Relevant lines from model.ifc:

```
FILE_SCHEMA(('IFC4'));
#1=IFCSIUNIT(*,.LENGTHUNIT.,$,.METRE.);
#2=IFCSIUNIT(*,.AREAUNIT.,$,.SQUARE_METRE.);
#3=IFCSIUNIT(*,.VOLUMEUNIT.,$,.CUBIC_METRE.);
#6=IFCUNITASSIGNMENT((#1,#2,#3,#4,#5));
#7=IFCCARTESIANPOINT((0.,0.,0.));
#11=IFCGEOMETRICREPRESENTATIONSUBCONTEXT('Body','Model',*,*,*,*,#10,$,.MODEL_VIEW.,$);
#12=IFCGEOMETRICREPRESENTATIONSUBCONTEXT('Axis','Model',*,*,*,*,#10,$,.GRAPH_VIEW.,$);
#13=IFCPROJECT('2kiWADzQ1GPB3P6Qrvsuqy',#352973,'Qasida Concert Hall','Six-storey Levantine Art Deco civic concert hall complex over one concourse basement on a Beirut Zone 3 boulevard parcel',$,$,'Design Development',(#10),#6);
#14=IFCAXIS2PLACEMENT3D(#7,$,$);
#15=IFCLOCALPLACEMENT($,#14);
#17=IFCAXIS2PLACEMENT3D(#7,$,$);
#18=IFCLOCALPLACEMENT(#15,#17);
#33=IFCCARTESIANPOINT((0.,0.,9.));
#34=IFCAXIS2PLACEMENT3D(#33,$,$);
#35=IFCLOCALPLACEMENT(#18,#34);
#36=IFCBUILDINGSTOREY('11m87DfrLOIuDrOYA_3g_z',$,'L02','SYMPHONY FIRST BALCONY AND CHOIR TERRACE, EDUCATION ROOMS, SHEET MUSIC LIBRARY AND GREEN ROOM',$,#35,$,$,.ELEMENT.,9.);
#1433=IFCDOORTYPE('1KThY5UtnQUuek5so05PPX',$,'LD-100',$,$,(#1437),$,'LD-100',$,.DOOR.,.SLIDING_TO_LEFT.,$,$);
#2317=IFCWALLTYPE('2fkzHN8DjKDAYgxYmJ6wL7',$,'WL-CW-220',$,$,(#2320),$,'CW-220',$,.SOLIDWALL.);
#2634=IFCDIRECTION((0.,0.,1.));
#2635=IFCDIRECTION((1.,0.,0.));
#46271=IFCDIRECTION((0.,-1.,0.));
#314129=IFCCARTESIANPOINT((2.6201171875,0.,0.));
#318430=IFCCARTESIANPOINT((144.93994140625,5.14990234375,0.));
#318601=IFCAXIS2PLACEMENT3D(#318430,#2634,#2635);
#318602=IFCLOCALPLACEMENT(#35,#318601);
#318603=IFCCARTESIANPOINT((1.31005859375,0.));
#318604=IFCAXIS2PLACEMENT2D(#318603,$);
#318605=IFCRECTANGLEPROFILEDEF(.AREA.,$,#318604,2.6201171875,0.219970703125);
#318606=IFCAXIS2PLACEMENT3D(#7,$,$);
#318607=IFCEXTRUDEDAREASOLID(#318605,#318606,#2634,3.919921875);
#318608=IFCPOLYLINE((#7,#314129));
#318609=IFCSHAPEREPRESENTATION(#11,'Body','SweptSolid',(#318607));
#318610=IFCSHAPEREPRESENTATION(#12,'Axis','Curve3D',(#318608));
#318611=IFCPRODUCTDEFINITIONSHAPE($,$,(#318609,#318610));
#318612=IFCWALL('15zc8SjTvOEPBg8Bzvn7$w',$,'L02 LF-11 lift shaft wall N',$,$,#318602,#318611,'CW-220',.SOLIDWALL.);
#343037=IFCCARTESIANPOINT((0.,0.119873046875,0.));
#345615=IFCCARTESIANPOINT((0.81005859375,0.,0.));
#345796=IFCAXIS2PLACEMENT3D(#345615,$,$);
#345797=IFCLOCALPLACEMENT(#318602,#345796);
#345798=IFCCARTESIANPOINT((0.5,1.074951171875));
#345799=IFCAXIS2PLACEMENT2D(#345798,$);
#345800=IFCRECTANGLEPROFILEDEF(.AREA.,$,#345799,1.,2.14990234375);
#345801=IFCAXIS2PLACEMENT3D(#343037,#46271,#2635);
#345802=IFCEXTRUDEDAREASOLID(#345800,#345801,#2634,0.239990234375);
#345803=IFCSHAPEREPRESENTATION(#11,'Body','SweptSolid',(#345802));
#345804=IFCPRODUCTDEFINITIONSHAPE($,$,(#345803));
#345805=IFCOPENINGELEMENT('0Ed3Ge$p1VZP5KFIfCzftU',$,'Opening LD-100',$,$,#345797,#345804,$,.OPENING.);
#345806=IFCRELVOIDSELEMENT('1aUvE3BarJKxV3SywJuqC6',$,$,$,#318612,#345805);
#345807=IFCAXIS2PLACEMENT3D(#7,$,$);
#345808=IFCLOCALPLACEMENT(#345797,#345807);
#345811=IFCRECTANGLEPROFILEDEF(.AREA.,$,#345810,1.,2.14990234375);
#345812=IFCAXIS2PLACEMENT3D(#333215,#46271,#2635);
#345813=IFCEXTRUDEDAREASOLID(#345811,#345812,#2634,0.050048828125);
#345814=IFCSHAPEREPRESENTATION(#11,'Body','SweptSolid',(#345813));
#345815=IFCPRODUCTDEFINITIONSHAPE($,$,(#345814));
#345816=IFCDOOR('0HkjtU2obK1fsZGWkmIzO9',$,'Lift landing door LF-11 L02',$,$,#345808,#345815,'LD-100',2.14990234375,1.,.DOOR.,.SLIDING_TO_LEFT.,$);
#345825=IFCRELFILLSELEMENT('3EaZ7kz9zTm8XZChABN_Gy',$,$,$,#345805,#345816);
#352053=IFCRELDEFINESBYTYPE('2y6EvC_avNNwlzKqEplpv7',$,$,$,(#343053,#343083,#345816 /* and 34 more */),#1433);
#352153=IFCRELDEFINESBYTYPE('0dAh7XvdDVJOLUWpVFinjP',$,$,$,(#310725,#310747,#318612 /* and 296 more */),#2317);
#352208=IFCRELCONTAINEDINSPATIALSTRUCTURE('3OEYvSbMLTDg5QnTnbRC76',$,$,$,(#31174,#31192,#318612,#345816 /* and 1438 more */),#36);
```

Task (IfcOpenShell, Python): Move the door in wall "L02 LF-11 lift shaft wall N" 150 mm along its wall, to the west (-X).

```python
import ifcopenshell
import ifcopenshell.api.geometry
import ifcopenshell.util.placement

model = ifcopenshell.open("model.ifc")

door = model.by_guid("0HkjtU2obK1fsZGWkmIzO9")
opening = door.FillsVoids[0].RelatingOpeningElement
wall = opening.VoidsElements[0].RelatingBuildingElement

wall_matrix = ifcopenshell.util.placement.get_local_placement(wall.ObjectPlacement)
shift = wall_matrix[:3, 0] * -0.15
before = ifcopenshell.util.placement.get_local_placement(door.ObjectPlacement)[:3, 3].copy()

# The door is placed relative to its opening, so it follows when the opening moves.
matrix = ifcopenshell.util.placement.get_local_placement(opening.ObjectPlacement)
matrix[:3, 3] += shift
ifcopenshell.api.geometry.edit_object_placement(
    model, product=opening, matrix=matrix, is_si=False, should_transform_children=True
)

after = ifcopenshell.util.placement.get_local_placement(door.ObjectPlacement)[:3, 3]
print("door moved by", (after - before).round(3) + 0.0)

model.write("model_rev.ifc")
```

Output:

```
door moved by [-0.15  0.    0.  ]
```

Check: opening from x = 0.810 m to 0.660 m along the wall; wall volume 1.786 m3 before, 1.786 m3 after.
